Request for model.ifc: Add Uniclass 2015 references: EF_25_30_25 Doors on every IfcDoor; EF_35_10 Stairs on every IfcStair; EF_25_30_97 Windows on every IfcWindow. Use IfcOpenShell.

First a look at what the model holds.

```python
import ifcopenshell

model = ifcopenshell.open("model.ifc")
print(model.schema)
print("classifications:", [c.Name for c in model.by_type("IfcClassification")])
for ifc_class in ("IfcDoor", "IfcRoof", "IfcStair", "IfcWall", "IfcWindow"):
    print(ifc_class, len(model.by_type(ifc_class)))
```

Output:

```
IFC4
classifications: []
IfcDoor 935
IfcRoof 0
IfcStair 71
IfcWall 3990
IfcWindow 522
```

```python
import ifcopenshell
import ifcopenshell.api.classification

model = ifcopenshell.open("model.ifc")

system = ifcopenshell.api.classification.add_classification(model, classification="Uniclass 2015")

codes = {
    "IfcDoor": ("EF_25_30_25", "Doors"),
    "IfcStair": ("EF_35_10", "Stairs"),
    "IfcWindow": ("EF_25_30_97", "Windows"),
}
for ifc_class, (code, name) in codes.items():
    products = model.by_type(ifc_class)
    ifcopenshell.api.classification.add_reference(
        model, products=products, classification=system, identification=code, name=name
    )
    print(code, len(products))

model.write("model_rev.ifc")
```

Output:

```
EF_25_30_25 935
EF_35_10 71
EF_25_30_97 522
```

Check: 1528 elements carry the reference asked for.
